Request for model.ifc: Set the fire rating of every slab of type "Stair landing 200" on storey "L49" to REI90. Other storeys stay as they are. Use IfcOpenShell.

First a look at what the model holds.

```python
import ifcopenshell
import ifcopenshell.util.element

model = ifcopenshell.open("model.ifc")
print(model.schema)
storey = next(s for s in model.by_type("IfcBuildingStorey") if s.Name == "L49")
slabs = [e for e in ifcopenshell.util.element.get_decomposition(storey) if e.is_a("IfcSlab")]
seen = {}
for e in slabs:
    element_type = ifcopenshell.util.element.get_type(e)
    key = (element_type.Name if element_type != e and element_type else None, ifcopenshell.util.element.get_pset(e, "Pset_SlabCommon", "FireRating"))
    seen[key] = seen.get(key, 0) + 1
for (name, value), count in sorted(seen.items(), key=str):
    print(count, "x", name, "|", value)
```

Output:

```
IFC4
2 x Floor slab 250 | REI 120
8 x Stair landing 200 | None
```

```python
import ifcopenshell
import ifcopenshell.api.pset
import ifcopenshell.util.element

model = ifcopenshell.open("model.ifc")

storey = next(s for s in model.by_type("IfcBuildingStorey") if s.Name == "L49")
slabs = [e for e in ifcopenshell.util.element.get_decomposition(storey) if e.is_a("IfcSlab")]

count = 0
for e in slabs:
    element_type = ifcopenshell.util.element.get_type(e)
    if element_type in (None, e) or element_type.Name != "Stair landing 200":
        continue
    found = ifcopenshell.util.element.get_pset(e, "Pset_SlabCommon", should_inherit=False)
    if found:
        pset = model.by_id(found["id"])
        if len(ifcopenshell.util.element.get_elements_by_pset(pset)) > 1:
            pset = ifcopenshell.api.pset.unshare_pset(model, products=[e], pset=pset)[0]
    else:
        pset = ifcopenshell.api.pset.add_pset(model, product=e, name="Pset_SlabCommon")
    ifcopenshell.api.pset.edit_pset(model, pset=pset, properties={"FireRating": "REI90"})
    count += 1

print(count, "slabs updated")

model.write("model_rev.ifc")
```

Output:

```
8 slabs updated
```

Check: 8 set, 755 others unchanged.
